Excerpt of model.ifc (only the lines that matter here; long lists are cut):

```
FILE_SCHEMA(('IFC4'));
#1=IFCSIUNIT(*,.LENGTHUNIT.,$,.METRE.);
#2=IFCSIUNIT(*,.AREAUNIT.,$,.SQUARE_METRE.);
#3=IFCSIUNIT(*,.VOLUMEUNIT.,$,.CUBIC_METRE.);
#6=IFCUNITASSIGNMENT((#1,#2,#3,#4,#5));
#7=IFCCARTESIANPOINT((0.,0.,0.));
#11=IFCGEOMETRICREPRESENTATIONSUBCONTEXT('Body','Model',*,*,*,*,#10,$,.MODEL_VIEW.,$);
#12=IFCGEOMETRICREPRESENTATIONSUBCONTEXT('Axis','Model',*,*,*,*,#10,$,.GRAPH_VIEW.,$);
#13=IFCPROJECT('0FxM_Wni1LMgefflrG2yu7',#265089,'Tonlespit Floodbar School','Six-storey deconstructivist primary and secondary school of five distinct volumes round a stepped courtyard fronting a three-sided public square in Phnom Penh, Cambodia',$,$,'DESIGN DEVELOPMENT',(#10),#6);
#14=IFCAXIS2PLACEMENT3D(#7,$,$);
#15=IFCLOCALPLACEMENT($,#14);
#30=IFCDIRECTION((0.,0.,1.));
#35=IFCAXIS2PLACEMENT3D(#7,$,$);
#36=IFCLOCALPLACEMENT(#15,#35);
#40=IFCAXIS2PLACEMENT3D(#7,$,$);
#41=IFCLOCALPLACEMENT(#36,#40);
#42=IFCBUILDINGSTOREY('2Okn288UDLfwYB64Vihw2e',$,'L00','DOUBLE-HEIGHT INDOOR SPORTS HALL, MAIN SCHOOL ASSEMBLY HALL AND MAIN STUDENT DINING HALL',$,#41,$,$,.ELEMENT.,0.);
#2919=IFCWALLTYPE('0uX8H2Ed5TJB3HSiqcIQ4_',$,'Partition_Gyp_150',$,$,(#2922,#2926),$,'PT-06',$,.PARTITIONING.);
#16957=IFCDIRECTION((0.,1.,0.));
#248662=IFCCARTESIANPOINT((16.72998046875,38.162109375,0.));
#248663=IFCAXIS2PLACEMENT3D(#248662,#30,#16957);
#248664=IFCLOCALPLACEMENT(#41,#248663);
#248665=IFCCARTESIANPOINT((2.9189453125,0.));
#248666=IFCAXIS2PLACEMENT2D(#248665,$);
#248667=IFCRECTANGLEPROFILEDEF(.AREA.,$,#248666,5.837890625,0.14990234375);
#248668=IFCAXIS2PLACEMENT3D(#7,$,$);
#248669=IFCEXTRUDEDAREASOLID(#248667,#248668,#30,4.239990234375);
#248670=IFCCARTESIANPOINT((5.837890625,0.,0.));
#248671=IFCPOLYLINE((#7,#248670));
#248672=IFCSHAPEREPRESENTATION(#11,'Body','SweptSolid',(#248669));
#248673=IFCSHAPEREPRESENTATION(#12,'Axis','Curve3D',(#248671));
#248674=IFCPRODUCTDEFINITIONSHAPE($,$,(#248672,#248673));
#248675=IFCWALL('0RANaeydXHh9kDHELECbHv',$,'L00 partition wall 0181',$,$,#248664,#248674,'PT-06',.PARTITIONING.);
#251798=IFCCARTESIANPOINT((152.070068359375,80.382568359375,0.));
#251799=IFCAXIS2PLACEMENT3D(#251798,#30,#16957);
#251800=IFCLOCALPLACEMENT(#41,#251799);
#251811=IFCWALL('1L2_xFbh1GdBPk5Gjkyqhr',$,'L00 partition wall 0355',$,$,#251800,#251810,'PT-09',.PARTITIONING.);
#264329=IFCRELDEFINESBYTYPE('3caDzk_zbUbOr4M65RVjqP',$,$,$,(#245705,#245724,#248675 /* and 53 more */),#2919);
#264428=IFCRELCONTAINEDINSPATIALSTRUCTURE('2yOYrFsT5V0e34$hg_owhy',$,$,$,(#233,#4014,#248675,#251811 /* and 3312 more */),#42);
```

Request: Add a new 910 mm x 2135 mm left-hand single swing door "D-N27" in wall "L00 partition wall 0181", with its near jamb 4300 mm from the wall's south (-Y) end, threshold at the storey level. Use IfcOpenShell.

```python
import numpy as np
import ifcopenshell
import ifcopenshell.api.feature
import ifcopenshell.api.geometry
import ifcopenshell.api.root
import ifcopenshell.api.spatial
import ifcopenshell.geom
import ifcopenshell.util.element
import ifcopenshell.util.placement
import ifcopenshell.util.representation
import ifcopenshell.util.shape
import ifcopenshell.util.unit

model = ifcopenshell.open("model.ifc")
unit_scale = ifcopenshell.util.unit.calculate_unit_scale(model)
settings = ifcopenshell.geom.settings()


def volume(element):
    """Net volume in cubic metres, openings subtracted."""
    shape = ifcopenshell.geom.create_shape(settings, element)
    return ifcopenshell.util.shape.get_volume(shape.geometry)


wall = model.by_guid("0RANaeydXHh9kDHELECbHv")
storey = ifcopenshell.util.element.get_container(wall, ifc_class="IfcBuildingStorey")
context = ifcopenshell.util.representation.get_context(model, "Model", "Body", "MODEL_VIEW")
before = volume(wall)

width, height, from_end, sill = 0.91, 2.135, 4.3, 0.0  # metres

# The wall runs along its own X axis, and the end named is its -X end.
wall_shape = ifcopenshell.geom.create_shape(settings, wall)
x, y, z = ifcopenshell.util.shape.get_vertices(wall_shape.geometry).T
start = x.min() + from_end
face, thickness = float(y.min()), float(y.max() - y.min())
wall_matrix = ifcopenshell.util.placement.get_local_placement(wall.ObjectPlacement)
level = ifcopenshell.util.placement.get_local_placement(storey.ObjectPlacement)[2, 3]


def in_wall(x, y):
    """Placement at x, y metres in the wall's axes, at sill height."""
    matrix = wall_matrix.copy()
    matrix[:, 3] = wall_matrix @ np.array([x / unit_scale, y / unit_scale, 0.0, 1.0])
    matrix[2, 3] = level + sill / unit_scale
    return matrix


# Opening: a box that overshoots both wall faces by 50 mm.
opening = ifcopenshell.api.root.create_entity(model, ifc_class="IfcOpeningElement", predefined_type="OPENING")
box = ifcopenshell.api.geometry.add_wall_representation(
    model, context=context, length=width, height=height, thickness=thickness + 0.1
)
ifcopenshell.api.geometry.assign_representation(model, product=opening, representation=box)
ifcopenshell.api.geometry.edit_object_placement(model, product=opening, matrix=in_wall(start, face - 0.05), is_si=False)
ifcopenshell.api.feature.add_feature(model, feature=opening, element=wall)

door = ifcopenshell.api.root.create_entity(model, ifc_class="IfcDoor", name="D-N27", predefined_type="DOOR")
door.OverallWidth, door.OverallHeight = width / unit_scale, height / unit_scale
door.OperationType = "SINGLE_SWING_LEFT"
body = ifcopenshell.api.geometry.add_door_representation(
    model,
    context=context,
    overall_width=door.OverallWidth,
    overall_height=door.OverallHeight,
    operation_type="SINGLE_SWING_LEFT",
    lining_properties={"LiningDepth": thickness / unit_scale, "ThresholdDepth": thickness / unit_scale},
)
ifcopenshell.api.geometry.assign_representation(model, product=door, representation=body)
ifcopenshell.api.spatial.assign_container(model, products=[door], relating_structure=storey)
ifcopenshell.api.feature.add_filling(model, opening=opening, element=door)

# The lining spans the wall, so the door starts at the wall face.
ifcopenshell.api.geometry.edit_object_placement(model, product=door, matrix=in_wall(start, face), is_si=False)

after = volume(wall)

print(f"wall volume {before:.3f} -> {after:.3f} m3")

model.write("model_rev.ifc")
```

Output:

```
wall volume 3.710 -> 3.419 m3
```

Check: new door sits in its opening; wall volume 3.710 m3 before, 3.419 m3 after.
